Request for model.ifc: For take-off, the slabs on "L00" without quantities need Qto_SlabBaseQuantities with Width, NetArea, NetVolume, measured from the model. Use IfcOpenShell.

First a look at what the model holds.

```python
import ifcopenshell
import ifcopenshell.util.element
import ifcopenshell.util.unit

model = ifcopenshell.open("model.ifc")
print(model.schema)
for unit_type in ("LENGTHUNIT", "AREAUNIT", "VOLUMEUNIT"):
    print(unit_type, ifcopenshell.util.unit.calculate_unit_scale(model, unit_type))
storey = next(s for s in model.by_type("IfcBuildingStorey") if s.Name == "L00")
slabs = [e for e in ifcopenshell.util.element.get_decomposition(storey) if e.is_a("IfcSlab")]
for e in sorted(slabs, key=lambda e: e.id()):
    print(e.id(), e.is_a(), e.Name, list(ifcopenshell.util.element.get_psets(e, qtos_only=True)), sep=" | ")
```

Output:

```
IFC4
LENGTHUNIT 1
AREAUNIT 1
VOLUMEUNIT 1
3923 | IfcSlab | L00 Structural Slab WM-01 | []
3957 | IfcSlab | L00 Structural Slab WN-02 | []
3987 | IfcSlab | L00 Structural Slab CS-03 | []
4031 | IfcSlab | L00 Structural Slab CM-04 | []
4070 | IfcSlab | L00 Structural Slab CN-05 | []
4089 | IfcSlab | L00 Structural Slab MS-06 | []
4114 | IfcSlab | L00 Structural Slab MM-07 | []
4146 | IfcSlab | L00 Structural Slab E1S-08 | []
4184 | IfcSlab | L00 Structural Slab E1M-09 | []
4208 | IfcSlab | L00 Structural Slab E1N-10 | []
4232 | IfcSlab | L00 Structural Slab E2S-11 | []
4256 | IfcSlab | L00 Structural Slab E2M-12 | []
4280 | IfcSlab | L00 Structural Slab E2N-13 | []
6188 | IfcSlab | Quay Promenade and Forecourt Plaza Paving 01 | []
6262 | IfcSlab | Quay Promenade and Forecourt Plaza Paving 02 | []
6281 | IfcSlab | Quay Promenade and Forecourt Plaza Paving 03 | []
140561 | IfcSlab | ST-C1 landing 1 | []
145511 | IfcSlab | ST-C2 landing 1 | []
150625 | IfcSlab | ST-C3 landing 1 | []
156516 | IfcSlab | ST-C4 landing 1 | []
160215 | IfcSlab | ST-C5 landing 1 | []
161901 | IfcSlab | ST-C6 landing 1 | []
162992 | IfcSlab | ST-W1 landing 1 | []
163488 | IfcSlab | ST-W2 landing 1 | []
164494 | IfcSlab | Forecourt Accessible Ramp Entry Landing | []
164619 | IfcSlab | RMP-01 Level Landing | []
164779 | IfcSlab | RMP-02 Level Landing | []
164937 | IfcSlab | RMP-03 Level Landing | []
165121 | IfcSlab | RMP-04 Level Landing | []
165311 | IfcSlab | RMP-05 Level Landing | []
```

```python
import ifcopenshell
import ifcopenshell.api.pset
import ifcopenshell.geom
import ifcopenshell.util.element
import ifcopenshell.util.shape
import ifcopenshell.util.unit

model = ifcopenshell.open("model.ifc")
unit_scale = ifcopenshell.util.unit.calculate_unit_scale(model)
area_scale = ifcopenshell.util.unit.calculate_unit_scale(model, "AREAUNIT")
volume_scale = ifcopenshell.util.unit.calculate_unit_scale(model, "VOLUMEUNIT")
settings = ifcopenshell.geom.settings()

storey = next(s for s in model.by_type("IfcBuildingStorey") if s.Name == "L00")
slabs = [e for e in ifcopenshell.util.element.get_decomposition(storey) if e.is_a("IfcSlab")]

for e in sorted(slabs, key=lambda e: e.id()):
    if ifcopenshell.util.element.get_psets(e, qtos_only=True, should_inherit=False):
        continue
    # Geometry comes back in metres, in the element's own axes.
    shape = ifcopenshell.geom.create_shape(settings, e)
    values = {
        "Width": ifcopenshell.util.shape.get_z(shape.geometry) / unit_scale,
        "NetArea": ifcopenshell.util.shape.get_footprint_area(shape.geometry) / area_scale,
        "NetVolume": ifcopenshell.util.shape.get_volume(shape.geometry) / volume_scale,
    }
    qto = ifcopenshell.api.pset.add_qto(model, product=e, name="Qto_SlabBaseQuantities")
    ifcopenshell.api.pset.edit_qto(model, qto=qto, properties=values)
    print(e.id(), {k: round(v, 3) for k, v in values.items()})

model.write("model_updated.ifc")
```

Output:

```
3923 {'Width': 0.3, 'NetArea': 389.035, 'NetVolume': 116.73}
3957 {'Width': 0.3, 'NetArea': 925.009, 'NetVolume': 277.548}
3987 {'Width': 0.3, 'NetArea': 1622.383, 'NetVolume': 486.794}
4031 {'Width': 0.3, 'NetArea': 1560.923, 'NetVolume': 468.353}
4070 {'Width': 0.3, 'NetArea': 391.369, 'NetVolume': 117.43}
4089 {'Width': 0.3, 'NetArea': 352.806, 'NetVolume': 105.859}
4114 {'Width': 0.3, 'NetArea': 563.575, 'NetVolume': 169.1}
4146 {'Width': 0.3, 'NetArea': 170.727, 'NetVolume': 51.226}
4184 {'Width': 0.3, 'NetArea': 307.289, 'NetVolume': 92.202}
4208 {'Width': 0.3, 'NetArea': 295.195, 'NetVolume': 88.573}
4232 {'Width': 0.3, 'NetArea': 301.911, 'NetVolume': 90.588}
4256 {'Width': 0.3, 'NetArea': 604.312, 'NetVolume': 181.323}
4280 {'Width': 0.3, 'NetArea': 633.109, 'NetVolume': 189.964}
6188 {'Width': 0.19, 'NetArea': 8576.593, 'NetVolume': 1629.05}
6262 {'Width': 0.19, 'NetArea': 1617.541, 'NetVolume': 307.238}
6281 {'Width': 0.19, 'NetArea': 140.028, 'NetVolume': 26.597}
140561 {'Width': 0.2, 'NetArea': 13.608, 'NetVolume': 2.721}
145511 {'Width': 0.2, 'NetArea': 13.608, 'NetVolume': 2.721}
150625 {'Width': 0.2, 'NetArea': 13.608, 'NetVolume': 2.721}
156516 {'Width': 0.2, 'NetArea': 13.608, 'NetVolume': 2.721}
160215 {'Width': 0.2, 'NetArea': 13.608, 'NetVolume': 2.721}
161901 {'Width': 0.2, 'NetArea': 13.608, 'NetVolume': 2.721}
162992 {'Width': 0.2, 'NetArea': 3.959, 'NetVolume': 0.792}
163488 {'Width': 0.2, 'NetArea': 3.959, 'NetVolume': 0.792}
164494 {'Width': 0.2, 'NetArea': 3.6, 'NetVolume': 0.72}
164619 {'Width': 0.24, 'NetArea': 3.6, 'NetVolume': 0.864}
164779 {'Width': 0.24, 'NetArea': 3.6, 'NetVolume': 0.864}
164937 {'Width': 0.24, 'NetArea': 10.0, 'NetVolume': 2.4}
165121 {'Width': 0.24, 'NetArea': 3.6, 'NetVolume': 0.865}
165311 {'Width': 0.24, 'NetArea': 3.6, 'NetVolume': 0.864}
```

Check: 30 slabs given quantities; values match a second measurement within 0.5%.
